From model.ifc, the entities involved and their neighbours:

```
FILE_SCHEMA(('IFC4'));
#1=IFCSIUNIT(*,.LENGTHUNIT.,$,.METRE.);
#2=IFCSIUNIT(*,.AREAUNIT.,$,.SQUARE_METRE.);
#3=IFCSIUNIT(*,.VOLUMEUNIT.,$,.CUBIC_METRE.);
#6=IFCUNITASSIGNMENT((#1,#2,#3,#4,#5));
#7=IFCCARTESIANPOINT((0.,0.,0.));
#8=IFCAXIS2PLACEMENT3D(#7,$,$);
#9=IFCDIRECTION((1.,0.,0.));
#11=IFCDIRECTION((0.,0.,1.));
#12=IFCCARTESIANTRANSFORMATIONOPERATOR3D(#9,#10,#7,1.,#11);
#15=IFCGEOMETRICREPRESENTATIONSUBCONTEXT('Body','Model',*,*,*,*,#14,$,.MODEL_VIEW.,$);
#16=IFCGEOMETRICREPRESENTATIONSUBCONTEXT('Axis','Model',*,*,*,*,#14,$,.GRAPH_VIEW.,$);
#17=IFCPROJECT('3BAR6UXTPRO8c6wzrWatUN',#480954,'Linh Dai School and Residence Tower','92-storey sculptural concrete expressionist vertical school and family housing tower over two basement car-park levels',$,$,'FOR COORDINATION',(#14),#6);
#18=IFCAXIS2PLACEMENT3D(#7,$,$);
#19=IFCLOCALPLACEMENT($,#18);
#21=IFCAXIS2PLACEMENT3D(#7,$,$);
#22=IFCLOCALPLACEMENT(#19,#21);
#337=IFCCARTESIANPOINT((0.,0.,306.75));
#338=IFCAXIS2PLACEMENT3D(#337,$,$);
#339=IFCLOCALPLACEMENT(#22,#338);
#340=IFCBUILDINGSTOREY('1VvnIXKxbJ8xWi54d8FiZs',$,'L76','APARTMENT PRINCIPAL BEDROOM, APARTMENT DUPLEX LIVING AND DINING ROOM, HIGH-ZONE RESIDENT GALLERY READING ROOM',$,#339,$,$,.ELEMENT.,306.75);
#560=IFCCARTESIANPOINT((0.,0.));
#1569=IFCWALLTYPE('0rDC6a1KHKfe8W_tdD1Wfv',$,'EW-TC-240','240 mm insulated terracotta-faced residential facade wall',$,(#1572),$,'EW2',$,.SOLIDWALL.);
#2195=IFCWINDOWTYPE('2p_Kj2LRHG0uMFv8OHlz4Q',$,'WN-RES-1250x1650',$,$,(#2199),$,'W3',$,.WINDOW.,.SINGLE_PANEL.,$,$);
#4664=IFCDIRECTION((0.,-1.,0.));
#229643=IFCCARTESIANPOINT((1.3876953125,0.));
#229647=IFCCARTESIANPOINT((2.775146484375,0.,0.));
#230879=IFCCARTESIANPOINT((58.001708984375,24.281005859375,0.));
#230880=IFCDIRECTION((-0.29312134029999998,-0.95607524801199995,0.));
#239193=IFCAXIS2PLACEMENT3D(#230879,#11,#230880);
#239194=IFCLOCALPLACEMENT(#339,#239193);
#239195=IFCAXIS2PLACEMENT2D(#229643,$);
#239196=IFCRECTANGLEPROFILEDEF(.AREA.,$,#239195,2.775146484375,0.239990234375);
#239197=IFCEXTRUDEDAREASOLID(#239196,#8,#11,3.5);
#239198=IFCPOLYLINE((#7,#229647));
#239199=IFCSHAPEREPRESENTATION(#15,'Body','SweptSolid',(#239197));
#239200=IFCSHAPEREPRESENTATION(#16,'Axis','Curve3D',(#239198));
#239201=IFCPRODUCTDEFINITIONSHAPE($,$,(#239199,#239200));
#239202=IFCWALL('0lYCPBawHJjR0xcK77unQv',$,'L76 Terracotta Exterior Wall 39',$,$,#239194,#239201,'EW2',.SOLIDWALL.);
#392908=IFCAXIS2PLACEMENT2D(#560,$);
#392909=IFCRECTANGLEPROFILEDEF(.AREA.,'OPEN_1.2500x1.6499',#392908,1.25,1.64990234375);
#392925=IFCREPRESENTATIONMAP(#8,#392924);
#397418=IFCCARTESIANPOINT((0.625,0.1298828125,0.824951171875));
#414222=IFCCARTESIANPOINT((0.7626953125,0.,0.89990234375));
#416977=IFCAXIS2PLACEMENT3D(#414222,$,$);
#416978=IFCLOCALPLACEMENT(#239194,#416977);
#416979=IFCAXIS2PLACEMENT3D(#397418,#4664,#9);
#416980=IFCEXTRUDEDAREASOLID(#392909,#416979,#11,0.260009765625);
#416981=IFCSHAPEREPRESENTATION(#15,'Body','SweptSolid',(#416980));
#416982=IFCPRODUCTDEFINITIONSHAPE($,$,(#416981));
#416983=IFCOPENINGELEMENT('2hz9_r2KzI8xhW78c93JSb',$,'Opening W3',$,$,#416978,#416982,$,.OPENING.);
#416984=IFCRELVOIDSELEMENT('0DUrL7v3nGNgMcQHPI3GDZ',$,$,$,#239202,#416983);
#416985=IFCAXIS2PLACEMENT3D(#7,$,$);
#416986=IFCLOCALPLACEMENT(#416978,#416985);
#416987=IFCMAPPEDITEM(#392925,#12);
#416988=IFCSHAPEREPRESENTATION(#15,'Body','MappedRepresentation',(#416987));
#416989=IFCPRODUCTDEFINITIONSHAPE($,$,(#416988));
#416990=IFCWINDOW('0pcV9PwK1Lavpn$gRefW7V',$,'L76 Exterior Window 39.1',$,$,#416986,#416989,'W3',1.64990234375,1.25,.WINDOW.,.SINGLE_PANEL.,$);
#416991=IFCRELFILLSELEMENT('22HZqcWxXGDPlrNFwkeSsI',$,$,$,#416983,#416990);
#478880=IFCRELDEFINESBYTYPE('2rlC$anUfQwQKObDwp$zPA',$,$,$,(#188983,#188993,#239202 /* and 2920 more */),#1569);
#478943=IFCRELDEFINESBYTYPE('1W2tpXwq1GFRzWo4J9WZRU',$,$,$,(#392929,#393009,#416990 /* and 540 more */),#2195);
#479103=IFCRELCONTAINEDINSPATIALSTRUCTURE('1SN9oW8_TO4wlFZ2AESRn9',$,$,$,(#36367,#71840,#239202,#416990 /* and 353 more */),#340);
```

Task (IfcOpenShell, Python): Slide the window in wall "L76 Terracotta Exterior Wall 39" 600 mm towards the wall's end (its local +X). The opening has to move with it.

```python
import ifcopenshell
import ifcopenshell.api.geometry
import ifcopenshell.util.placement
import ifcopenshell.util.unit

model = ifcopenshell.open("model.ifc")
unit_scale = ifcopenshell.util.unit.calculate_unit_scale(model)

window = model.by_guid("0pcV9PwK1Lavpn$gRefW7V")
opening = window.FillsVoids[0].RelatingOpeningElement
wall = opening.VoidsElements[0].RelatingBuildingElement

wall_matrix = ifcopenshell.util.placement.get_local_placement(wall.ObjectPlacement)
shift = wall_matrix[:3, 0] * 0.6 / unit_scale
before = ifcopenshell.util.placement.get_local_placement(window.ObjectPlacement)[:3, 3].copy()

# The window is placed relative to its opening, so it follows when the opening moves.
matrix = ifcopenshell.util.placement.get_local_placement(opening.ObjectPlacement)
matrix[:3, 3] += shift
ifcopenshell.api.geometry.edit_object_placement(
    model, product=opening, matrix=matrix, is_si=False, should_transform_children=True
)

after = ifcopenshell.util.placement.get_local_placement(window.ObjectPlacement)[:3, 3]
print("window moved by", (after - before).round(3) + 0.0)

model.write("model_rev.ifc")
```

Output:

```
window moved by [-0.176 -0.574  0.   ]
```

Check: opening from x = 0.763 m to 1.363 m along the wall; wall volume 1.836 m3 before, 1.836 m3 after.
